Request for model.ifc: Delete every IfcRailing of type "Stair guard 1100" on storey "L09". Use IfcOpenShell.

First a look at what the model holds.

```python
import ifcopenshell
import ifcopenshell.util.element

model = ifcopenshell.open("model.ifc")
print(model.schema)
storey = next(s for s in model.by_type("IfcBuildingStorey") if s.Name == "L09")
railings = [e for e in ifcopenshell.util.element.get_decomposition(storey) if e.is_a("IfcRailing")]
seen = {}
for e in railings:
    element_type = ifcopenshell.util.element.get_type(e)
    name = element_type.Name if element_type not in (None, e) else None
    seen[name] = seen.get(name, 0) + 1
for name, count in sorted(seen.items(), key=str):
    print(count, "x", name)
```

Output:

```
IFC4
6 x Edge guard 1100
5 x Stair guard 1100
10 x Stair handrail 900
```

```python
import ifcopenshell
import ifcopenshell.api.root
import ifcopenshell.util.element

model = ifcopenshell.open("model.ifc")

storey = next(s for s in model.by_type("IfcBuildingStorey") if s.Name == "L09")
railings = [e for e in ifcopenshell.util.element.get_decomposition(storey) if e.is_a("IfcRailing")]
targets = [e for e in railings if (t := ifcopenshell.util.element.get_type(e)) not in (None, e) and t.Name == "Stair guard 1100"]

for e in targets:
    ifcopenshell.api.root.remove_product(model, product=e)
print(len(targets), "removed")

model.write("model_edited.ifc")
```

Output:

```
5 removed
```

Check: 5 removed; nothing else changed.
